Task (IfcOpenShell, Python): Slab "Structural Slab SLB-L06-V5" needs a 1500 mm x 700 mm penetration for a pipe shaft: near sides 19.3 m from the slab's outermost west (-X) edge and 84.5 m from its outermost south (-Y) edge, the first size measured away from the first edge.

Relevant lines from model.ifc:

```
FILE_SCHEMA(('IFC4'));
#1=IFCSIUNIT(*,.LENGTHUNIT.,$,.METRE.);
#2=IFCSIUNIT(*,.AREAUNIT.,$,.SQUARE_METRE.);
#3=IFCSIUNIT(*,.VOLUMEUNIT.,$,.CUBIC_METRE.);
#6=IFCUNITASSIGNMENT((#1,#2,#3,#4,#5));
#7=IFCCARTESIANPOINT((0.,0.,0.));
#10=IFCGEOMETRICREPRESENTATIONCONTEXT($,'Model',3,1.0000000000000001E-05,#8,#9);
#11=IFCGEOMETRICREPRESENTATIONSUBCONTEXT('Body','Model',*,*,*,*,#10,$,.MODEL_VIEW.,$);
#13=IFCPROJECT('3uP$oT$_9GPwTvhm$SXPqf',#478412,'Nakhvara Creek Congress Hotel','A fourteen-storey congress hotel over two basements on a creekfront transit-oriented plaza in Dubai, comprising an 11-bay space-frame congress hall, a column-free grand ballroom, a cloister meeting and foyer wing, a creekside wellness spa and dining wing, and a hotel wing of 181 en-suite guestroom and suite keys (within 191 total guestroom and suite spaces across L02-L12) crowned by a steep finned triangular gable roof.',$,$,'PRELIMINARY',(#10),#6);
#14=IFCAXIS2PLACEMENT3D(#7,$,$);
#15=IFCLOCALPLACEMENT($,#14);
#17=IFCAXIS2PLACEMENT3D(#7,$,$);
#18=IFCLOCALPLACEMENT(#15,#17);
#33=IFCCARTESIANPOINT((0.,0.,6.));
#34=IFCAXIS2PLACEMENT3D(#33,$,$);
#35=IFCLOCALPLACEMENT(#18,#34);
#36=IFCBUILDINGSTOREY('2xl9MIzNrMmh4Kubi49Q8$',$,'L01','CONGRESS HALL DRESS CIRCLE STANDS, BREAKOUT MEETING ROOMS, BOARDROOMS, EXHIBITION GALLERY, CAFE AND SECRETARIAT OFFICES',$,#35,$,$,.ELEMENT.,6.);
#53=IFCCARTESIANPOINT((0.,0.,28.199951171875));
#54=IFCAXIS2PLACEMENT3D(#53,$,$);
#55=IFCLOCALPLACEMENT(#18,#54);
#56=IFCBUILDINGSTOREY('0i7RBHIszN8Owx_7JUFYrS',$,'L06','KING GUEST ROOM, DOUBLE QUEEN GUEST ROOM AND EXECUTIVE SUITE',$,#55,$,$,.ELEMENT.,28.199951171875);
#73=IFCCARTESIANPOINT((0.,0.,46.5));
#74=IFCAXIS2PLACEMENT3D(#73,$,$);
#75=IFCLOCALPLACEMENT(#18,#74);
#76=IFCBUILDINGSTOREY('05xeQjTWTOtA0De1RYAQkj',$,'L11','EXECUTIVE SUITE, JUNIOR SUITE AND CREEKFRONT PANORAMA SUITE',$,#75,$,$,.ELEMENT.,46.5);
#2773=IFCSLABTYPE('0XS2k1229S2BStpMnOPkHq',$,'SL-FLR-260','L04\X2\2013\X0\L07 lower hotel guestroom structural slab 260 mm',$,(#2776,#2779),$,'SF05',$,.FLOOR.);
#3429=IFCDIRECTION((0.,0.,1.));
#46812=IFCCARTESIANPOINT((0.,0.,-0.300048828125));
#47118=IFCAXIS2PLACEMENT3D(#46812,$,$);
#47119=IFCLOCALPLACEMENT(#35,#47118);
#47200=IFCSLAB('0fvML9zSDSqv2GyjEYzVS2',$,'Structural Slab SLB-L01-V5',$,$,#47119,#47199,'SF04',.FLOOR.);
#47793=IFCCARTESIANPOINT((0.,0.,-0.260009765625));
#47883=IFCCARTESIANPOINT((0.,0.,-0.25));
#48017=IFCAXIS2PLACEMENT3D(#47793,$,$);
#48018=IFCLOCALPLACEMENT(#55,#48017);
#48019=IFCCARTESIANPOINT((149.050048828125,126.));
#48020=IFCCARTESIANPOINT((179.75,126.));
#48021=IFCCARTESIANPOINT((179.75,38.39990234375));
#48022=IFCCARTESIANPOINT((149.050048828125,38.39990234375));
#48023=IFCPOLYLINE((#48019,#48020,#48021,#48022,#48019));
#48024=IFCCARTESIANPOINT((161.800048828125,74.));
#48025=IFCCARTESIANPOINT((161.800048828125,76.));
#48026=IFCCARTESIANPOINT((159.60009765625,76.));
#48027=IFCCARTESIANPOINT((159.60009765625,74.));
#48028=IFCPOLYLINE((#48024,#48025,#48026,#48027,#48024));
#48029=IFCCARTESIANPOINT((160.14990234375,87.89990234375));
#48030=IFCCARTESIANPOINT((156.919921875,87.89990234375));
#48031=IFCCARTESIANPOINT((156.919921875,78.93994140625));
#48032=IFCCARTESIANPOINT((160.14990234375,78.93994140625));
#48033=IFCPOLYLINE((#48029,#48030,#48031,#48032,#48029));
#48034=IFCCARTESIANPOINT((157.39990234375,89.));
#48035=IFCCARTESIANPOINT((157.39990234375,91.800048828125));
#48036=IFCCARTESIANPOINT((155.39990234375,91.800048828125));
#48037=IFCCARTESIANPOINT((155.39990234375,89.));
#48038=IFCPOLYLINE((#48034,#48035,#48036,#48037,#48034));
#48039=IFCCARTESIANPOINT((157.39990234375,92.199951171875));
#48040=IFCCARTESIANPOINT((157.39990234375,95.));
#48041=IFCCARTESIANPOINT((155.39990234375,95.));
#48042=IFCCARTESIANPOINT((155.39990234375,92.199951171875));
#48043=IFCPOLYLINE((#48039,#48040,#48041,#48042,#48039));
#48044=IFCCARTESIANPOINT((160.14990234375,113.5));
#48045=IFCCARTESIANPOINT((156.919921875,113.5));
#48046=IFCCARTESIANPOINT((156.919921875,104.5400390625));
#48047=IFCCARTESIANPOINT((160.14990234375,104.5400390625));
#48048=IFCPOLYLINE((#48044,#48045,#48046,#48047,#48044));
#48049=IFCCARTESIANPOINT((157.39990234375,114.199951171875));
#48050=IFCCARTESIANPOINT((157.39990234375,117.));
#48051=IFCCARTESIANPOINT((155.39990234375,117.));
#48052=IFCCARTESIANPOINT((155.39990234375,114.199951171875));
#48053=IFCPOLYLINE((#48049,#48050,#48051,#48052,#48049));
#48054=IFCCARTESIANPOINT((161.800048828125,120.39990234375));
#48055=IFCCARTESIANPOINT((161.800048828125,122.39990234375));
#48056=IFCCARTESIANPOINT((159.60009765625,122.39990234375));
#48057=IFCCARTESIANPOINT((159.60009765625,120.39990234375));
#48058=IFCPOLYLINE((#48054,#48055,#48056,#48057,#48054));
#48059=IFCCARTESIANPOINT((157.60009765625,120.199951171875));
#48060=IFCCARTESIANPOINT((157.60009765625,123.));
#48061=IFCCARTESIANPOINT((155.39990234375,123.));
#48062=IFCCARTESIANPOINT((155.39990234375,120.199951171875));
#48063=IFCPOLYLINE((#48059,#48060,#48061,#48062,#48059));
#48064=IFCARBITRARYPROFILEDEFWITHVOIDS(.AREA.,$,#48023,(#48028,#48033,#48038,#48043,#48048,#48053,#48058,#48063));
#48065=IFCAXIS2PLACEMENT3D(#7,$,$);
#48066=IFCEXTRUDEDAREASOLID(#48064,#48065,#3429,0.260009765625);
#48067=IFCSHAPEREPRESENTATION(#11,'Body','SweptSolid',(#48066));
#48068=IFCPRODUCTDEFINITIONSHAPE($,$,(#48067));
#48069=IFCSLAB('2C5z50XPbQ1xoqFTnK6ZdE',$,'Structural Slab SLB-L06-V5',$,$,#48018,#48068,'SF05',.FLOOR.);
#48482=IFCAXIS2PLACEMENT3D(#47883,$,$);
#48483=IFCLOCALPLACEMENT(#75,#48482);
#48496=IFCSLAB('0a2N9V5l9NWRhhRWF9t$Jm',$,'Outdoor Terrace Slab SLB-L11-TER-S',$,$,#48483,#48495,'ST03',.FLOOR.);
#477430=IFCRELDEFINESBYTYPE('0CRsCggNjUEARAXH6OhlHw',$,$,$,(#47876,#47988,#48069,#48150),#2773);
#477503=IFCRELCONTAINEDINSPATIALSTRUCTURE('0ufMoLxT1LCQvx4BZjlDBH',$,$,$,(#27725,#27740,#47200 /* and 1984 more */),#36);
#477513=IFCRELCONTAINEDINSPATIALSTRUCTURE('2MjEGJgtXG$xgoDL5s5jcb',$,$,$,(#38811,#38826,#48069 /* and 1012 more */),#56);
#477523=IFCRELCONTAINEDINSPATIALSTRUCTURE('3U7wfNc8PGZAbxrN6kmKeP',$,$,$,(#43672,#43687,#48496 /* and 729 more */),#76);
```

```python
import numpy as np
import ifcopenshell
import ifcopenshell.api.feature
import ifcopenshell.api.geometry
import ifcopenshell.api.root
import ifcopenshell.geom
import ifcopenshell.util.placement
import ifcopenshell.util.representation
import ifcopenshell.util.shape
import ifcopenshell.util.unit

model = ifcopenshell.open("model.ifc")
unit_scale = ifcopenshell.util.unit.calculate_unit_scale(model)
settings = ifcopenshell.geom.settings()


def volume(element):
    """Net volume in cubic metres, openings subtracted."""
    shape = ifcopenshell.geom.create_shape(settings, element)
    return ifcopenshell.util.shape.get_volume(shape.geometry)


slab = model.by_id(48069)
before = volume(slab)

# Extent in the slab's own axes, in metres. The edges named are its -X and -Y sides.
slab_shape = ifcopenshell.geom.create_shape(settings, slab)
vertices = ifcopenshell.util.shape.get_vertices(slab_shape.geometry)
x_min, y_min, bottom = vertices.min(axis=0)
top = vertices[:, 2].max()

opening = ifcopenshell.api.root.create_entity(model, ifc_class="IfcOpeningElement", name="Pipe shaft opening", predefined_type="OPENING")
context = ifcopenshell.util.representation.get_context(model, "Model", "Body", "MODEL_VIEW")
width, depth = 1.5, 0.7
outline = [(0.0, 0.0), (width, 0.0), (width, depth), (0.0, depth), (0.0, 0.0)]
# Overshoot both faces by 50 mm so the cut is clean.
shape = ifcopenshell.api.geometry.add_slab_representation(
    model, context=context, depth=top - bottom + 0.1, polyline=outline
)
ifcopenshell.api.geometry.assign_representation(model, product=opening, representation=shape)

matrix = ifcopenshell.util.placement.get_local_placement(slab.ObjectPlacement)
matrix[:, 3] = matrix @ np.append(np.array([x_min + 19.3, y_min + 84.5, bottom - 0.05]) / unit_scale, 1.0)
ifcopenshell.api.geometry.edit_object_placement(model, product=opening, matrix=matrix, is_si=False)
ifcopenshell.api.feature.add_feature(model, feature=opening, element=slab)

after = volume(slab)

print(f"slab volume {before:.3f} -> {after:.3f} m3")

model.write("model_updated.ifc")
```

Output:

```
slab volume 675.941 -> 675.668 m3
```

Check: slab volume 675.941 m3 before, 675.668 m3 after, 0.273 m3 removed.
